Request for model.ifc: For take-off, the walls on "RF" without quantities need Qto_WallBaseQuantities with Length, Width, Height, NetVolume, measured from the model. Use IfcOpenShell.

First a look at what the model holds.

```python
import ifcopenshell
import ifcopenshell.util.element
import ifcopenshell.util.unit

model = ifcopenshell.open("model.ifc")
print(model.schema)
for unit_type in ("LENGTHUNIT", "AREAUNIT", "VOLUMEUNIT"):
    print(unit_type, ifcopenshell.util.unit.calculate_unit_scale(model, unit_type))
storey = next(s for s in model.by_type("IfcBuildingStorey") if s.Name == "RF")
walls = [e for e in ifcopenshell.util.element.get_decomposition(storey) if e.is_a("IfcWall")]
for e in sorted(walls, key=lambda e: e.id()):
    print(e.id(), e.is_a(), e.Name, list(ifcopenshell.util.element.get_psets(e, qtos_only=True)), sep=" | ")
```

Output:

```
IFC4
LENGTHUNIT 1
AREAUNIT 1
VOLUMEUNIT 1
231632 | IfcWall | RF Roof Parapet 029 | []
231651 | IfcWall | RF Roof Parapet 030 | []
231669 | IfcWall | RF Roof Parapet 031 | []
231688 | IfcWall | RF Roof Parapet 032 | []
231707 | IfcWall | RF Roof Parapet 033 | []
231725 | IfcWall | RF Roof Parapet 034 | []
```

```python
import ifcopenshell
import ifcopenshell.api.pset
import ifcopenshell.geom
import ifcopenshell.util.element
import ifcopenshell.util.shape
import ifcopenshell.util.unit

model = ifcopenshell.open("model.ifc")
unit_scale = ifcopenshell.util.unit.calculate_unit_scale(model)
volume_scale = ifcopenshell.util.unit.calculate_unit_scale(model, "VOLUMEUNIT")
settings = ifcopenshell.geom.settings()

storey = next(s for s in model.by_type("IfcBuildingStorey") if s.Name == "RF")
walls = [e for e in ifcopenshell.util.element.get_decomposition(storey) if e.is_a("IfcWall")]

for e in sorted(walls, key=lambda e: e.id()):
    if ifcopenshell.util.element.get_psets(e, qtos_only=True, should_inherit=False):
        continue
    # Geometry comes back in metres, in the element's own axes.
    shape = ifcopenshell.geom.create_shape(settings, e)
    values = {
        "Length": ifcopenshell.util.shape.get_x(shape.geometry) / unit_scale,
        "Width": ifcopenshell.util.shape.get_y(shape.geometry) / unit_scale,
        "Height": ifcopenshell.util.shape.get_z(shape.geometry) / unit_scale,
        "NetVolume": ifcopenshell.util.shape.get_volume(shape.geometry) / volume_scale,
    }
    qto = ifcopenshell.api.pset.add_qto(model, product=e, name="Qto_WallBaseQuantities")
    ifcopenshell.api.pset.edit_qto(model, qto=qto, properties=values)
    print(e.id(), {k: round(v, 3) for k, v in values.items()})

model.write("model_updated.ifc")
```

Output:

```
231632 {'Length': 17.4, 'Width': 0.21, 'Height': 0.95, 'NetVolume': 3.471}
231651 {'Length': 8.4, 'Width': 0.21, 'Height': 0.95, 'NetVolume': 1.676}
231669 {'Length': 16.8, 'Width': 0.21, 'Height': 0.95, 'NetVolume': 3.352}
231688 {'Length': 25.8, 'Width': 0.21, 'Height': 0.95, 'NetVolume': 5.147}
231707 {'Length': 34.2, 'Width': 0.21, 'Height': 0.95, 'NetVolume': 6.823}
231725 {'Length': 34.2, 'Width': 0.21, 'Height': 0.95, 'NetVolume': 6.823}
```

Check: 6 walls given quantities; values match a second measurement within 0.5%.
